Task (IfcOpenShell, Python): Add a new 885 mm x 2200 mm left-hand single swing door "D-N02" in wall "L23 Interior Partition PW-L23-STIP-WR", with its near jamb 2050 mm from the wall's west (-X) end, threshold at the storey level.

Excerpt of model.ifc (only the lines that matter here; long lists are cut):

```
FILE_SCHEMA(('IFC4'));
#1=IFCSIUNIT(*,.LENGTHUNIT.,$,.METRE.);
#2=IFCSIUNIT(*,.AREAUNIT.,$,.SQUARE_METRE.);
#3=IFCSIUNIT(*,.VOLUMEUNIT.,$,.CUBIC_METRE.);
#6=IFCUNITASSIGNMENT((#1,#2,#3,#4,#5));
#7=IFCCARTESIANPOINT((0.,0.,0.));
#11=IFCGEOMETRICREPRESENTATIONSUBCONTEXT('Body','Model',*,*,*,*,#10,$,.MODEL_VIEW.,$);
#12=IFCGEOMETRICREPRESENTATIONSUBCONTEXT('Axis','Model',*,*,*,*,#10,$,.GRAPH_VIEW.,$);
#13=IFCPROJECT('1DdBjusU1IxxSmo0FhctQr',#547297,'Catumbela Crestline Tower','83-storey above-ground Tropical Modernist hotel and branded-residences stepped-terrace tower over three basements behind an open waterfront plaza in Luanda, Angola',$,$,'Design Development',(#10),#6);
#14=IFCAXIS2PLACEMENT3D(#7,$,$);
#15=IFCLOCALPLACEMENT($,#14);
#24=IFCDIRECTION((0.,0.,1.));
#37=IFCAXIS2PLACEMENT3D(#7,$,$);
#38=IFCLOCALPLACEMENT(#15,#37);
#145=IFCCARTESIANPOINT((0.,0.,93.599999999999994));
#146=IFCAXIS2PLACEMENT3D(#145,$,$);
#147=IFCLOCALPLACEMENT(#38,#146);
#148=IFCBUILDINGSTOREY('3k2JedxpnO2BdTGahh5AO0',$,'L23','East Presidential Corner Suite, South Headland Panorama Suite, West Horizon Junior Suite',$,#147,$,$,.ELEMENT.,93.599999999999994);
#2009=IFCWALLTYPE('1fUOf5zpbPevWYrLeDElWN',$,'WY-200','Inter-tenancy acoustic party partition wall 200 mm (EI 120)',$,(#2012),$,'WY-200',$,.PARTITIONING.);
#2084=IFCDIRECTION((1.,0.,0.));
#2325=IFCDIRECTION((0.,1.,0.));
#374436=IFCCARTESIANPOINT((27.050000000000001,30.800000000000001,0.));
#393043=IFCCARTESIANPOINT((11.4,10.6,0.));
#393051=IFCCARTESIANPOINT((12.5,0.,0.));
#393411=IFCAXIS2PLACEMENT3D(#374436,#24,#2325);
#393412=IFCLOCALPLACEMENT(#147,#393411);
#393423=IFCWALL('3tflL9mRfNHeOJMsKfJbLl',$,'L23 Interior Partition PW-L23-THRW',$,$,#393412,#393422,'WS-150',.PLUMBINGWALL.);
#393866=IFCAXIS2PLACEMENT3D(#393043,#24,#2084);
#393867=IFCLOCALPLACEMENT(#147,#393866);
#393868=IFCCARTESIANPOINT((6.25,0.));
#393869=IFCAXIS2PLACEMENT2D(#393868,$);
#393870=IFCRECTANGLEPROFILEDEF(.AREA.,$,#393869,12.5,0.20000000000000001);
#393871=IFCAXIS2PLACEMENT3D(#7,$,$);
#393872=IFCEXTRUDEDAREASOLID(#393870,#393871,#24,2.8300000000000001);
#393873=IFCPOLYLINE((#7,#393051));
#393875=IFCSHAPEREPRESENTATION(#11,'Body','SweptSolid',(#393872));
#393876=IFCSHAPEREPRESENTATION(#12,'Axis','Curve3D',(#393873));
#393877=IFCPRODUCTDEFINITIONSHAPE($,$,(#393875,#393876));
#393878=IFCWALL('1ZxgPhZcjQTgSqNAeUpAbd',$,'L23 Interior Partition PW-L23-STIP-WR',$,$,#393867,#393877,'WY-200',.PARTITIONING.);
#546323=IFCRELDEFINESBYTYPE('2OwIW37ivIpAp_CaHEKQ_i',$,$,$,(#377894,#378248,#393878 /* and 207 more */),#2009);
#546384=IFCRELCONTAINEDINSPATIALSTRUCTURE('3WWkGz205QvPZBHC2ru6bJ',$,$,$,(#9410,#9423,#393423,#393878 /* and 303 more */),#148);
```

```python
import numpy as np
import ifcopenshell
import ifcopenshell.api.feature
import ifcopenshell.api.geometry
import ifcopenshell.api.root
import ifcopenshell.api.spatial
import ifcopenshell.geom
import ifcopenshell.util.element
import ifcopenshell.util.placement
import ifcopenshell.util.representation
import ifcopenshell.util.shape
import ifcopenshell.util.unit

model = ifcopenshell.open("model.ifc")
unit_scale = ifcopenshell.util.unit.calculate_unit_scale(model)
settings = ifcopenshell.geom.settings()


def volume(element):
    """Net volume in cubic metres, openings subtracted."""
    shape = ifcopenshell.geom.create_shape(settings, element)
    return ifcopenshell.util.shape.get_volume(shape.geometry)


wall = model.by_id(393878)
storey = ifcopenshell.util.element.get_container(wall, ifc_class="IfcBuildingStorey")
context = ifcopenshell.util.representation.get_context(model, "Model", "Body", "MODEL_VIEW")
before = volume(wall)

width, height, from_end, sill = 0.885, 2.2, 2.05, 0.0  # metres

# The wall runs along its own X axis, and the end named is its -X end.
wall_shape = ifcopenshell.geom.create_shape(settings, wall)
x, y, z = ifcopenshell.util.shape.get_vertices(wall_shape.geometry).T
start = x.min() + from_end
face, thickness = float(y.min()), float(y.max() - y.min())
wall_matrix = ifcopenshell.util.placement.get_local_placement(wall.ObjectPlacement)
level = ifcopenshell.util.placement.get_local_placement(storey.ObjectPlacement)[2, 3]


def in_wall(x, y):
    """Placement at x, y metres in the wall's axes, at sill height."""
    matrix = wall_matrix.copy()
    matrix[:, 3] = wall_matrix @ np.array([x / unit_scale, y / unit_scale, 0.0, 1.0])
    matrix[2, 3] = level + sill / unit_scale
    return matrix


# Opening: a box that overshoots both wall faces by 50 mm.
opening = ifcopenshell.api.root.create_entity(model, ifc_class="IfcOpeningElement", predefined_type="OPENING")
box = ifcopenshell.api.geometry.add_wall_representation(
    model, context=context, length=width, height=height, thickness=thickness + 0.1
)
ifcopenshell.api.geometry.assign_representation(model, product=opening, representation=box)
ifcopenshell.api.geometry.edit_object_placement(model, product=opening, matrix=in_wall(start, face - 0.05), is_si=False)
ifcopenshell.api.feature.add_feature(model, feature=opening, element=wall)

door = ifcopenshell.api.root.create_entity(model, ifc_class="IfcDoor", name="D-N02", predefined_type="DOOR")
door.OverallWidth, door.OverallHeight = width / unit_scale, height / unit_scale
door.OperationType = "SINGLE_SWING_LEFT"
body = ifcopenshell.api.geometry.add_door_representation(
    model,
    context=context,
    overall_width=door.OverallWidth,
    overall_height=door.OverallHeight,
    operation_type="SINGLE_SWING_LEFT",
    lining_properties={"LiningDepth": thickness / unit_scale, "ThresholdDepth": thickness / unit_scale},
)
ifcopenshell.api.geometry.assign_representation(model, product=door, representation=body)
ifcopenshell.api.spatial.assign_container(model, products=[door], relating_structure=storey)
ifcopenshell.api.feature.add_filling(model, opening=opening, element=door)

# The lining spans the wall, so the door starts at the wall face.
ifcopenshell.api.geometry.edit_object_placement(model, product=door, matrix=in_wall(start, face), is_si=False)

after = volume(wall)

print(f"wall volume {before:.3f} -> {after:.3f} m3")

model.write("model_rev.ifc")
```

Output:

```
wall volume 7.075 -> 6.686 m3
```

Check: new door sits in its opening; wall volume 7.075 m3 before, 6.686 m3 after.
